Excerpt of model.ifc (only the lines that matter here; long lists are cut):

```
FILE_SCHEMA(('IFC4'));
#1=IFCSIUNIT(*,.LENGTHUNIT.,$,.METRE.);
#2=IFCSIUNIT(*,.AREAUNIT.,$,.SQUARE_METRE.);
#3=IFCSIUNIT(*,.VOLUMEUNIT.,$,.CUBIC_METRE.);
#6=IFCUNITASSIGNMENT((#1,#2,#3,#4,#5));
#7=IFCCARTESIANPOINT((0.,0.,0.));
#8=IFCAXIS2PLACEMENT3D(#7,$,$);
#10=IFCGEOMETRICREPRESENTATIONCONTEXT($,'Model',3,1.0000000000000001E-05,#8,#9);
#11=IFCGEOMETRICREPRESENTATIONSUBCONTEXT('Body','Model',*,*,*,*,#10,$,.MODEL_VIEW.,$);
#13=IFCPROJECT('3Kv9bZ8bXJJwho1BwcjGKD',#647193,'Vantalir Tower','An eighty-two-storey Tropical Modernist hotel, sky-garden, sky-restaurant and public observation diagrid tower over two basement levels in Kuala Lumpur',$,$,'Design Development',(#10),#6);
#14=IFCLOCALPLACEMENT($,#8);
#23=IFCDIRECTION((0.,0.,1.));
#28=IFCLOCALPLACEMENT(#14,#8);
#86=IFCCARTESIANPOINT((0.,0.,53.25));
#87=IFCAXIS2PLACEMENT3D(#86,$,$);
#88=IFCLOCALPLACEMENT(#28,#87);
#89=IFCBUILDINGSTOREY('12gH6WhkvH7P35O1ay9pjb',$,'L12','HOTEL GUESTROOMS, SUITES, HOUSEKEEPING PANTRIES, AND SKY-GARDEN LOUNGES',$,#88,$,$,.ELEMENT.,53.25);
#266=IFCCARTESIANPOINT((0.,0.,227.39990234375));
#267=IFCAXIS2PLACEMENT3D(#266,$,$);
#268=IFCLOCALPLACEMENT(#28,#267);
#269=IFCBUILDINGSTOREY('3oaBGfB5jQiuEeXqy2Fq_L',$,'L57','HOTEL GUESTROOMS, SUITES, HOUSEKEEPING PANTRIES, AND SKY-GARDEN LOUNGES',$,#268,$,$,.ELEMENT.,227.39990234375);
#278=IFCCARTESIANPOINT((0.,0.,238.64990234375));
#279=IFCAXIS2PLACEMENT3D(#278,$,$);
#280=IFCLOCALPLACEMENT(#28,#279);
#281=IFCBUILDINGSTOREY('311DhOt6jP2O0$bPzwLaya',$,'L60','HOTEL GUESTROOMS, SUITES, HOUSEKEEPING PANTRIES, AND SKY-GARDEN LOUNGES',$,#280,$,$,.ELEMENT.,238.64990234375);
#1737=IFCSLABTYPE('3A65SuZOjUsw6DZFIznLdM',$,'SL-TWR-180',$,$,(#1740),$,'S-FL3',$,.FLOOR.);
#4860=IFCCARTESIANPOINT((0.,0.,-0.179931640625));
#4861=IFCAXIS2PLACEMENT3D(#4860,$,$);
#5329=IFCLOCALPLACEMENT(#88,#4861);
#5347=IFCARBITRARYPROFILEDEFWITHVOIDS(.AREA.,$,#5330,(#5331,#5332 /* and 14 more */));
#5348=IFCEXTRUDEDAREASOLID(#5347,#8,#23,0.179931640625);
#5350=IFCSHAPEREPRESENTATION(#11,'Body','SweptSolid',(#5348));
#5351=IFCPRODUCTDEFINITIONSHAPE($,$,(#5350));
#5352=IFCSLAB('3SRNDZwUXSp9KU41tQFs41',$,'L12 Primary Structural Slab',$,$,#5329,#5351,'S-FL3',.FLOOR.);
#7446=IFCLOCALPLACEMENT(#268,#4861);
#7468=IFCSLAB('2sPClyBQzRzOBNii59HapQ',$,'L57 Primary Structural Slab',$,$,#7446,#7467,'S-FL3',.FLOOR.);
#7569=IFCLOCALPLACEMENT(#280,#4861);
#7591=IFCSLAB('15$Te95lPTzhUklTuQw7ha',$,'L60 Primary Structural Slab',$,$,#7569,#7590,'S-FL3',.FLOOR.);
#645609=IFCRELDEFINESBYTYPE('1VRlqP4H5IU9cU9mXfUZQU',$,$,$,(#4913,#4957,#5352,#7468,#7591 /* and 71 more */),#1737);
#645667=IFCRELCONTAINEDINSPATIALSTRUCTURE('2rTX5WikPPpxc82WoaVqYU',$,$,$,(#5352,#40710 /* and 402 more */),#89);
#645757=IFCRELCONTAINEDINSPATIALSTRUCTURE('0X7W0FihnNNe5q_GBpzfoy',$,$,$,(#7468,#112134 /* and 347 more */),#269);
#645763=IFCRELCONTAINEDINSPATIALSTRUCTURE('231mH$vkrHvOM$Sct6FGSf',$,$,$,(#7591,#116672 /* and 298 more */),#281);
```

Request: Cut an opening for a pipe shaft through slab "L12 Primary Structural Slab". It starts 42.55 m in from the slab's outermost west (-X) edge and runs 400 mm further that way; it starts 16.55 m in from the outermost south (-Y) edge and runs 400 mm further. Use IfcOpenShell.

```python
import numpy as np
import ifcopenshell
import ifcopenshell.api.feature
import ifcopenshell.api.geometry
import ifcopenshell.api.root
import ifcopenshell.geom
import ifcopenshell.util.placement
import ifcopenshell.util.representation
import ifcopenshell.util.shape
import ifcopenshell.util.unit

model = ifcopenshell.open("model.ifc")
unit_scale = ifcopenshell.util.unit.calculate_unit_scale(model)
settings = ifcopenshell.geom.settings()


def volume(element):
    """Net volume in cubic metres, openings subtracted."""
    shape = ifcopenshell.geom.create_shape(settings, element)
    return ifcopenshell.util.shape.get_volume(shape.geometry)


slab = model.by_guid("3SRNDZwUXSp9KU41tQFs41")
before = volume(slab)

# Extent in the slab's own axes, in metres. The edges named are its -X and -Y sides.
slab_shape = ifcopenshell.geom.create_shape(settings, slab)
vertices = ifcopenshell.util.shape.get_vertices(slab_shape.geometry)
x_min, y_min, bottom = vertices.min(axis=0)
top = vertices[:, 2].max()

opening = ifcopenshell.api.root.create_entity(model, ifc_class="IfcOpeningElement", name="Pipe shaft opening", predefined_type="OPENING")
context = ifcopenshell.util.representation.get_context(model, "Model", "Body", "MODEL_VIEW")
width, depth = 0.4, 0.4
outline = [(0.0, 0.0), (width, 0.0), (width, depth), (0.0, depth), (0.0, 0.0)]
# Overshoot both faces by 50 mm so the cut is clean.
shape = ifcopenshell.api.geometry.add_slab_representation(
    model, context=context, depth=top - bottom + 0.1, polyline=outline
)
ifcopenshell.api.geometry.assign_representation(model, product=opening, representation=shape)

matrix = ifcopenshell.util.placement.get_local_placement(slab.ObjectPlacement)
matrix[:, 3] = matrix @ np.append(np.array([x_min + 42.55, y_min + 16.55, bottom - 0.05]) / unit_scale, 1.0)
ifcopenshell.api.geometry.edit_object_placement(model, product=opening, matrix=matrix, is_si=False)
ifcopenshell.api.feature.add_feature(model, feature=opening, element=slab)

after = volume(slab)

print(f"slab volume {before:.3f} -> {after:.3f} m3")

model.write("model_updated.ifc")
```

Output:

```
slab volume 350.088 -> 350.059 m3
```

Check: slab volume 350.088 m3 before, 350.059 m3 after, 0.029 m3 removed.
